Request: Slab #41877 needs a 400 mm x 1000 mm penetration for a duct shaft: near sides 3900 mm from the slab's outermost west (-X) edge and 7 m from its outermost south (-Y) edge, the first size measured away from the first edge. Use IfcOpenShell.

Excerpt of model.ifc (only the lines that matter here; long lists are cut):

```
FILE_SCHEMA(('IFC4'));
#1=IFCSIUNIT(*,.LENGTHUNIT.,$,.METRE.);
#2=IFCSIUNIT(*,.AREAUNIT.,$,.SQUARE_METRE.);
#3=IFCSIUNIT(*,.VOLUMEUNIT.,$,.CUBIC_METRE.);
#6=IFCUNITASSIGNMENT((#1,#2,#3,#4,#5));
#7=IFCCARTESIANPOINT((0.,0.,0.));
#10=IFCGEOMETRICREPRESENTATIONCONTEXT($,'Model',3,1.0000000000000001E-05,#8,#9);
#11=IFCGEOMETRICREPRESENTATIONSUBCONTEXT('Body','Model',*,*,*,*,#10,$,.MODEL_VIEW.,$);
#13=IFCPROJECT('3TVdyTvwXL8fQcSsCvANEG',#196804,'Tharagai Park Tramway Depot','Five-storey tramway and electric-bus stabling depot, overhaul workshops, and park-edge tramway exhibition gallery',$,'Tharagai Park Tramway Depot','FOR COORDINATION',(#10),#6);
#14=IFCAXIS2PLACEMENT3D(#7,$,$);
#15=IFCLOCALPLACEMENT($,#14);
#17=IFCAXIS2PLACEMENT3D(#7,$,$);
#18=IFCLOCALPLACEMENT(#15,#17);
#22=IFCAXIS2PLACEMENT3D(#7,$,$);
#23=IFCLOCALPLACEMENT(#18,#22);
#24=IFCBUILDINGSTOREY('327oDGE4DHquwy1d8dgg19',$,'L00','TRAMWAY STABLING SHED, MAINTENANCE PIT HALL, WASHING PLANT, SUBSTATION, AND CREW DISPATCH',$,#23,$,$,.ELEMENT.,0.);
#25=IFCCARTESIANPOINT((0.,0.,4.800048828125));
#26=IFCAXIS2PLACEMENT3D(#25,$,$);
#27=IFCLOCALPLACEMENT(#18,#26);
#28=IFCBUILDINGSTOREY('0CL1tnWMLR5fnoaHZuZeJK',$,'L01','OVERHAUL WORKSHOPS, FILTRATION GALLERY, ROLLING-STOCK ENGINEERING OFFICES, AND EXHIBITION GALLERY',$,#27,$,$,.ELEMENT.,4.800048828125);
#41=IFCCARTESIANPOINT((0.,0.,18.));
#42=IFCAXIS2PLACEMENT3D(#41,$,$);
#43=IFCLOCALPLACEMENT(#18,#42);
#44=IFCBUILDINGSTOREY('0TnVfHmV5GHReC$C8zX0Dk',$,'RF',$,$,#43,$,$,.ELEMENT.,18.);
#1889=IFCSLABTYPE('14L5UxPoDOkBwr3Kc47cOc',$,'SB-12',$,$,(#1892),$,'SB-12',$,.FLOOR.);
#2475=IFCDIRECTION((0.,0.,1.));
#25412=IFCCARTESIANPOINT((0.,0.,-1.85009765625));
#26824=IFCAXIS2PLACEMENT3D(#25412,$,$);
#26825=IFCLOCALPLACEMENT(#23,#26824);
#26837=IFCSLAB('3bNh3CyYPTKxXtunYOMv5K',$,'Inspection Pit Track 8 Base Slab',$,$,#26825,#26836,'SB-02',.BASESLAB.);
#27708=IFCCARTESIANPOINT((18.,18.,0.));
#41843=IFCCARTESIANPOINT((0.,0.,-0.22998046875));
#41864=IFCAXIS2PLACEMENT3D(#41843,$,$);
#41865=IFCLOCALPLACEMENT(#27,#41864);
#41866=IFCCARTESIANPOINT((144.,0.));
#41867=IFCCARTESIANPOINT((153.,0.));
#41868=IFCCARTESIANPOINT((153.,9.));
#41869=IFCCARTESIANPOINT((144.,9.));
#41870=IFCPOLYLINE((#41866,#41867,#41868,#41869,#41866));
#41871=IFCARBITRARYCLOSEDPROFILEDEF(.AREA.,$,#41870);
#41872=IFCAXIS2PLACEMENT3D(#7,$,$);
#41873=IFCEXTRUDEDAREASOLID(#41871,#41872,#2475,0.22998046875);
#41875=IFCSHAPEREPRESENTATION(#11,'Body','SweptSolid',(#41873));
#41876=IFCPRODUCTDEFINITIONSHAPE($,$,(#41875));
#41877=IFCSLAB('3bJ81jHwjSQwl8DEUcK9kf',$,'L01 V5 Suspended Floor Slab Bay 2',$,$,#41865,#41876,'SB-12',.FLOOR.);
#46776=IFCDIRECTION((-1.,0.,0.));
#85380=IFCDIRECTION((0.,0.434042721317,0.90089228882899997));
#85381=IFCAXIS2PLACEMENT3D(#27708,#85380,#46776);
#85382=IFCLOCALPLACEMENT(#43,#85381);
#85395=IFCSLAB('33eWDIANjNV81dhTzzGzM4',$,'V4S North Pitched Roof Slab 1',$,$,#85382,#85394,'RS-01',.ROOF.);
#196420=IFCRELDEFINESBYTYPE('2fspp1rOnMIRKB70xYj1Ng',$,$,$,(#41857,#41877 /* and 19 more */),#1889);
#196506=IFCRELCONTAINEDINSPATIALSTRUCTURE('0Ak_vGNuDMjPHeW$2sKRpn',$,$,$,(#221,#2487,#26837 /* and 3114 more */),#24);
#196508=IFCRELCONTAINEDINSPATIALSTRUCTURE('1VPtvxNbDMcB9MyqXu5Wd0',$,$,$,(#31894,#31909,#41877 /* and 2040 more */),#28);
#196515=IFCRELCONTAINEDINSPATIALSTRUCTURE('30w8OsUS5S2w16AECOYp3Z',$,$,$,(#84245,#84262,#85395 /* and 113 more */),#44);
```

```python
import numpy as np
import ifcopenshell
import ifcopenshell.api.feature
import ifcopenshell.api.geometry
import ifcopenshell.api.root
import ifcopenshell.geom
import ifcopenshell.util.placement
import ifcopenshell.util.representation
import ifcopenshell.util.shape
import ifcopenshell.util.unit

model = ifcopenshell.open("model.ifc")
unit_scale = ifcopenshell.util.unit.calculate_unit_scale(model)
settings = ifcopenshell.geom.settings()


def volume(element):
    """Net volume in cubic metres, openings subtracted."""
    shape = ifcopenshell.geom.create_shape(settings, element)
    return ifcopenshell.util.shape.get_volume(shape.geometry)


slab = model.by_id(41877)
before = volume(slab)

# Extent in the slab's own axes, in metres. The edges named are its -X and -Y sides.
slab_shape = ifcopenshell.geom.create_shape(settings, slab)
vertices = ifcopenshell.util.shape.get_vertices(slab_shape.geometry)
x_min, y_min, bottom = vertices.min(axis=0)
top = vertices[:, 2].max()

opening = ifcopenshell.api.root.create_entity(model, ifc_class="IfcOpeningElement", name="Duct shaft opening", predefined_type="OPENING")
context = ifcopenshell.util.representation.get_context(model, "Model", "Body", "MODEL_VIEW")
width, depth = 0.4, 1
outline = [(0.0, 0.0), (width, 0.0), (width, depth), (0.0, depth), (0.0, 0.0)]
# Overshoot both faces by 50 mm so the cut is clean.
shape = ifcopenshell.api.geometry.add_slab_representation(
    model, context=context, depth=top - bottom + 0.1, polyline=outline
)
ifcopenshell.api.geometry.assign_representation(model, product=opening, representation=shape)

matrix = ifcopenshell.util.placement.get_local_placement(slab.ObjectPlacement)
matrix[:, 3] = matrix @ np.append(np.array([x_min + 3.9, y_min + 7, bottom - 0.05]) / unit_scale, 1.0)
ifcopenshell.api.geometry.edit_object_placement(model, product=opening, matrix=matrix, is_si=False)
ifcopenshell.api.feature.add_feature(model, feature=opening, element=slab)

after = volume(slab)

print(f"slab volume {before:.3f} -> {after:.3f} m3")

model.write("model-out.ifc")
```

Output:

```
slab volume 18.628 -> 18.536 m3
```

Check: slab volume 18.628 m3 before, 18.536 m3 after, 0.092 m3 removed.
